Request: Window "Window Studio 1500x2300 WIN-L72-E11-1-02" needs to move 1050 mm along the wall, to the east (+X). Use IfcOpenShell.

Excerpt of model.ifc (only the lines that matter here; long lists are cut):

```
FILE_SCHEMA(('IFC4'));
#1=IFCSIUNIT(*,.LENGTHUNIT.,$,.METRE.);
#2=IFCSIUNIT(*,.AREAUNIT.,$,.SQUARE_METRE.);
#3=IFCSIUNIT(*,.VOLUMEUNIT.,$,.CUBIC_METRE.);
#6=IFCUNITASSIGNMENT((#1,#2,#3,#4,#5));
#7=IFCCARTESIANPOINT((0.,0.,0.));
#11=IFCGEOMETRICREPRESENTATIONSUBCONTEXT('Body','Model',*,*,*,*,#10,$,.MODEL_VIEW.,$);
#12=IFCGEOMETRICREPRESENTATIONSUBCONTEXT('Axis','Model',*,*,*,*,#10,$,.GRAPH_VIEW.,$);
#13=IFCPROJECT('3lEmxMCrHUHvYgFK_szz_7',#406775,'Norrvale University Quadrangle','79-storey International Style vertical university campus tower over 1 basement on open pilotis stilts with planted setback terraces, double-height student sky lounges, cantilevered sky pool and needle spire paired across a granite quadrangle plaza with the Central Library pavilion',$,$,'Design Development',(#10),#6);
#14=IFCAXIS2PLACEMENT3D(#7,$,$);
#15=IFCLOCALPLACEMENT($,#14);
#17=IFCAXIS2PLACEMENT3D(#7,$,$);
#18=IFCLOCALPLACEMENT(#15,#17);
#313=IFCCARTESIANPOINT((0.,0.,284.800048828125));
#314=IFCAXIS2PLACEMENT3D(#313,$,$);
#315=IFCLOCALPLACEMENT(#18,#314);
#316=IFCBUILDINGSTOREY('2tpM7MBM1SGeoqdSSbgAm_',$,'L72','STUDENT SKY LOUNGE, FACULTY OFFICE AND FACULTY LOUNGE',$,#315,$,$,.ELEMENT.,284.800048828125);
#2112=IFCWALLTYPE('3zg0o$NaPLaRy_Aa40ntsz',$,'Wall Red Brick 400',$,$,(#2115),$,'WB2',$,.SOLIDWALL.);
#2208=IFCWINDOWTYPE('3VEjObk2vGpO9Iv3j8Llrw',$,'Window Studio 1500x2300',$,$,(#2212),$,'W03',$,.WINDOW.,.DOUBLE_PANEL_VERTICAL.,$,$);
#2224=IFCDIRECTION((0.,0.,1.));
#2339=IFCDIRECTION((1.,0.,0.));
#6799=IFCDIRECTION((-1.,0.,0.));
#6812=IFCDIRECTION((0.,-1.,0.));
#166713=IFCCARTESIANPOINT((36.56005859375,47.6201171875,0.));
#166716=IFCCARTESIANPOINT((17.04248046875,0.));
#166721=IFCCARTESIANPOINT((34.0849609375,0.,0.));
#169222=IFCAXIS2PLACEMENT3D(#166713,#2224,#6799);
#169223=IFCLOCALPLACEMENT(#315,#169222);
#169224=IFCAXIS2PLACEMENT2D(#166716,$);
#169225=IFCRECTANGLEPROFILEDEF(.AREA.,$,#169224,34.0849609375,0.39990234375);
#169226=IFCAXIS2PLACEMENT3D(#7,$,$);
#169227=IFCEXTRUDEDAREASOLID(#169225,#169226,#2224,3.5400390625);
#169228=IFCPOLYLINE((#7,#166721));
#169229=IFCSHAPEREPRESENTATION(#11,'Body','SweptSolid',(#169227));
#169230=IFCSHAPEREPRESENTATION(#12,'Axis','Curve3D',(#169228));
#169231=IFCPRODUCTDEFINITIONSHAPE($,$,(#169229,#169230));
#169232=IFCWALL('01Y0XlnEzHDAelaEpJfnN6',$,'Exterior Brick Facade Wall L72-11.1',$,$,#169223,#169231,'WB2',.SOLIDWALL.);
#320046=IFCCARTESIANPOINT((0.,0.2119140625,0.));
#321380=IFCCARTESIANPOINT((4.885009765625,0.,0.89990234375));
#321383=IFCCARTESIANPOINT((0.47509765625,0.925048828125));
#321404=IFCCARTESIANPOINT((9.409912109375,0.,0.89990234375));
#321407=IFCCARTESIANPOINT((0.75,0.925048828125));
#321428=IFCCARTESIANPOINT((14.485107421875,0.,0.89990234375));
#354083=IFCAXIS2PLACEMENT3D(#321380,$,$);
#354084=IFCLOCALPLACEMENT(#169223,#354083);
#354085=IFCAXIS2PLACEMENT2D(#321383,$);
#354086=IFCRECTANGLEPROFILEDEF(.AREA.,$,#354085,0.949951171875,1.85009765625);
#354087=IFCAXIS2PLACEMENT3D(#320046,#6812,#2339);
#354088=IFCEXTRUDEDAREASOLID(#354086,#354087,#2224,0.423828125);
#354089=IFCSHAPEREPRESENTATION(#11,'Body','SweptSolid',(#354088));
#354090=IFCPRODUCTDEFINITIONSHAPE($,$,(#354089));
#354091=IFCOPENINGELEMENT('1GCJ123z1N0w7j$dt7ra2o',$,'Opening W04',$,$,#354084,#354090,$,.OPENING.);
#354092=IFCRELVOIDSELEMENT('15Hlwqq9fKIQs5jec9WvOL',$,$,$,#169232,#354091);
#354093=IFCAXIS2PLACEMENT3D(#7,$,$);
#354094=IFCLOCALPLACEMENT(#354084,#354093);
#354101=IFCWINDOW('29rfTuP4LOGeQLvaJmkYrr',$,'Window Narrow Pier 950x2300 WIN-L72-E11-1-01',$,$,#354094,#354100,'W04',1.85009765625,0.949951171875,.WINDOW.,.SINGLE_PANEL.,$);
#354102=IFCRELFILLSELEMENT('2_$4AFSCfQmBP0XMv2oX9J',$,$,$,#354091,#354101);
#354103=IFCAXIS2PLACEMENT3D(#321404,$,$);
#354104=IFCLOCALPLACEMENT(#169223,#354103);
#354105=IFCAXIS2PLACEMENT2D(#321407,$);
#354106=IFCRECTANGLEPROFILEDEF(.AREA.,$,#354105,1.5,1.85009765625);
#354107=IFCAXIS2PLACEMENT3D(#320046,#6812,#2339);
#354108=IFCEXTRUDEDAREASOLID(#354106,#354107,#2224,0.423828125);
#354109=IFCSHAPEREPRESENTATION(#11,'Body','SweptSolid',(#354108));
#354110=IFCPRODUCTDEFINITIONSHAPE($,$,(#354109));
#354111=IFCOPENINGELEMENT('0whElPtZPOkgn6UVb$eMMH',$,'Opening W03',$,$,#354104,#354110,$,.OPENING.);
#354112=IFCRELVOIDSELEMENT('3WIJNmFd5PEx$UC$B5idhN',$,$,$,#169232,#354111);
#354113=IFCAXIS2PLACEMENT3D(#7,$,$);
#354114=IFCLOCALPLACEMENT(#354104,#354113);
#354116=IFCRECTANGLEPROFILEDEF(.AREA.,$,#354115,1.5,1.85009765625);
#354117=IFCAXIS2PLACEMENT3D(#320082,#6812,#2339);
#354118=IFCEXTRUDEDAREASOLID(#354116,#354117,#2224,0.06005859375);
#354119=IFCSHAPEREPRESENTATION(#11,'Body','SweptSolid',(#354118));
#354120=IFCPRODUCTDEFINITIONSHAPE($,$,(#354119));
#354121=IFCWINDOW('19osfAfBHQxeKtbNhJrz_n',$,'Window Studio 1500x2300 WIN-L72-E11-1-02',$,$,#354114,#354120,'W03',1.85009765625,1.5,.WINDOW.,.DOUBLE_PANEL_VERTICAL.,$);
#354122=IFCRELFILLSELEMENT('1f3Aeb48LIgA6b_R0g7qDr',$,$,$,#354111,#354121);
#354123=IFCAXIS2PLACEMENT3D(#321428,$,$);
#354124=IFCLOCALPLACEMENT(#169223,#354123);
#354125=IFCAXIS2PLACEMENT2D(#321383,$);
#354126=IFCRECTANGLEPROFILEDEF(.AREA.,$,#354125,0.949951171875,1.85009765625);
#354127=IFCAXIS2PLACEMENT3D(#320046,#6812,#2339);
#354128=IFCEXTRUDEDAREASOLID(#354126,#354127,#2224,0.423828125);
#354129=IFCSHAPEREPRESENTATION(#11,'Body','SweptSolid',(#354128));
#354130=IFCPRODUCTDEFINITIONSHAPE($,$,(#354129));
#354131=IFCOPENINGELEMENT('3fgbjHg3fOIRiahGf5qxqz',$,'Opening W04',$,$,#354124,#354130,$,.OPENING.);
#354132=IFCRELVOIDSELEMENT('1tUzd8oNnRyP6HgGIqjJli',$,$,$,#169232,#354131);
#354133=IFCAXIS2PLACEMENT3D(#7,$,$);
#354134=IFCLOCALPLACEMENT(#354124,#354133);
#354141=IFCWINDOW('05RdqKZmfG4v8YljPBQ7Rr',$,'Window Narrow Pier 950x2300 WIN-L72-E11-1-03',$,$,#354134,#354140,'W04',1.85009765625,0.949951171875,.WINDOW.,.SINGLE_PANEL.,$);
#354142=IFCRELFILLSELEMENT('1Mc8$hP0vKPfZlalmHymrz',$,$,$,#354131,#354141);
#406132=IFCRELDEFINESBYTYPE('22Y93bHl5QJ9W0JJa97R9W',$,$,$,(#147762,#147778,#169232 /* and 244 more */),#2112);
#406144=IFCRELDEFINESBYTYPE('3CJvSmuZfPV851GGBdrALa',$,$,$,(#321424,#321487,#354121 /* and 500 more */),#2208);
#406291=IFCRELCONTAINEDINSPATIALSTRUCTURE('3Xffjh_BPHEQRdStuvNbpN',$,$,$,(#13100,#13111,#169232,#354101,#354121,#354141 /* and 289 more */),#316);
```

```python
import ifcopenshell
import ifcopenshell.api.geometry
import ifcopenshell.util.placement
import ifcopenshell.util.unit

model = ifcopenshell.open("model.ifc")
unit_scale = ifcopenshell.util.unit.calculate_unit_scale(model)

window = model.by_guid("19osfAfBHQxeKtbNhJrz_n")
opening = window.FillsVoids[0].RelatingOpeningElement
wall = opening.VoidsElements[0].RelatingBuildingElement

wall_matrix = ifcopenshell.util.placement.get_local_placement(wall.ObjectPlacement)
shift = wall_matrix[:3, 0] * -1.05 / unit_scale
before = ifcopenshell.util.placement.get_local_placement(window.ObjectPlacement)[:3, 3].copy()

# The window is placed relative to its opening, so it follows when the opening moves.
matrix = ifcopenshell.util.placement.get_local_placement(opening.ObjectPlacement)
matrix[:3, 3] += shift
ifcopenshell.api.geometry.edit_object_placement(
    model, product=opening, matrix=matrix, is_si=False, should_transform_children=True
)

after = ifcopenshell.util.placement.get_local_placement(window.ObjectPlacement)[:3, 3]
print("window moved by", (after - before).round(3) + 0.0)

model.write("model-out.ifc")
```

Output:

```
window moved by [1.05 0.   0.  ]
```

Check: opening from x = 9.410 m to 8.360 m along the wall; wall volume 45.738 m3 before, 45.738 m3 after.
